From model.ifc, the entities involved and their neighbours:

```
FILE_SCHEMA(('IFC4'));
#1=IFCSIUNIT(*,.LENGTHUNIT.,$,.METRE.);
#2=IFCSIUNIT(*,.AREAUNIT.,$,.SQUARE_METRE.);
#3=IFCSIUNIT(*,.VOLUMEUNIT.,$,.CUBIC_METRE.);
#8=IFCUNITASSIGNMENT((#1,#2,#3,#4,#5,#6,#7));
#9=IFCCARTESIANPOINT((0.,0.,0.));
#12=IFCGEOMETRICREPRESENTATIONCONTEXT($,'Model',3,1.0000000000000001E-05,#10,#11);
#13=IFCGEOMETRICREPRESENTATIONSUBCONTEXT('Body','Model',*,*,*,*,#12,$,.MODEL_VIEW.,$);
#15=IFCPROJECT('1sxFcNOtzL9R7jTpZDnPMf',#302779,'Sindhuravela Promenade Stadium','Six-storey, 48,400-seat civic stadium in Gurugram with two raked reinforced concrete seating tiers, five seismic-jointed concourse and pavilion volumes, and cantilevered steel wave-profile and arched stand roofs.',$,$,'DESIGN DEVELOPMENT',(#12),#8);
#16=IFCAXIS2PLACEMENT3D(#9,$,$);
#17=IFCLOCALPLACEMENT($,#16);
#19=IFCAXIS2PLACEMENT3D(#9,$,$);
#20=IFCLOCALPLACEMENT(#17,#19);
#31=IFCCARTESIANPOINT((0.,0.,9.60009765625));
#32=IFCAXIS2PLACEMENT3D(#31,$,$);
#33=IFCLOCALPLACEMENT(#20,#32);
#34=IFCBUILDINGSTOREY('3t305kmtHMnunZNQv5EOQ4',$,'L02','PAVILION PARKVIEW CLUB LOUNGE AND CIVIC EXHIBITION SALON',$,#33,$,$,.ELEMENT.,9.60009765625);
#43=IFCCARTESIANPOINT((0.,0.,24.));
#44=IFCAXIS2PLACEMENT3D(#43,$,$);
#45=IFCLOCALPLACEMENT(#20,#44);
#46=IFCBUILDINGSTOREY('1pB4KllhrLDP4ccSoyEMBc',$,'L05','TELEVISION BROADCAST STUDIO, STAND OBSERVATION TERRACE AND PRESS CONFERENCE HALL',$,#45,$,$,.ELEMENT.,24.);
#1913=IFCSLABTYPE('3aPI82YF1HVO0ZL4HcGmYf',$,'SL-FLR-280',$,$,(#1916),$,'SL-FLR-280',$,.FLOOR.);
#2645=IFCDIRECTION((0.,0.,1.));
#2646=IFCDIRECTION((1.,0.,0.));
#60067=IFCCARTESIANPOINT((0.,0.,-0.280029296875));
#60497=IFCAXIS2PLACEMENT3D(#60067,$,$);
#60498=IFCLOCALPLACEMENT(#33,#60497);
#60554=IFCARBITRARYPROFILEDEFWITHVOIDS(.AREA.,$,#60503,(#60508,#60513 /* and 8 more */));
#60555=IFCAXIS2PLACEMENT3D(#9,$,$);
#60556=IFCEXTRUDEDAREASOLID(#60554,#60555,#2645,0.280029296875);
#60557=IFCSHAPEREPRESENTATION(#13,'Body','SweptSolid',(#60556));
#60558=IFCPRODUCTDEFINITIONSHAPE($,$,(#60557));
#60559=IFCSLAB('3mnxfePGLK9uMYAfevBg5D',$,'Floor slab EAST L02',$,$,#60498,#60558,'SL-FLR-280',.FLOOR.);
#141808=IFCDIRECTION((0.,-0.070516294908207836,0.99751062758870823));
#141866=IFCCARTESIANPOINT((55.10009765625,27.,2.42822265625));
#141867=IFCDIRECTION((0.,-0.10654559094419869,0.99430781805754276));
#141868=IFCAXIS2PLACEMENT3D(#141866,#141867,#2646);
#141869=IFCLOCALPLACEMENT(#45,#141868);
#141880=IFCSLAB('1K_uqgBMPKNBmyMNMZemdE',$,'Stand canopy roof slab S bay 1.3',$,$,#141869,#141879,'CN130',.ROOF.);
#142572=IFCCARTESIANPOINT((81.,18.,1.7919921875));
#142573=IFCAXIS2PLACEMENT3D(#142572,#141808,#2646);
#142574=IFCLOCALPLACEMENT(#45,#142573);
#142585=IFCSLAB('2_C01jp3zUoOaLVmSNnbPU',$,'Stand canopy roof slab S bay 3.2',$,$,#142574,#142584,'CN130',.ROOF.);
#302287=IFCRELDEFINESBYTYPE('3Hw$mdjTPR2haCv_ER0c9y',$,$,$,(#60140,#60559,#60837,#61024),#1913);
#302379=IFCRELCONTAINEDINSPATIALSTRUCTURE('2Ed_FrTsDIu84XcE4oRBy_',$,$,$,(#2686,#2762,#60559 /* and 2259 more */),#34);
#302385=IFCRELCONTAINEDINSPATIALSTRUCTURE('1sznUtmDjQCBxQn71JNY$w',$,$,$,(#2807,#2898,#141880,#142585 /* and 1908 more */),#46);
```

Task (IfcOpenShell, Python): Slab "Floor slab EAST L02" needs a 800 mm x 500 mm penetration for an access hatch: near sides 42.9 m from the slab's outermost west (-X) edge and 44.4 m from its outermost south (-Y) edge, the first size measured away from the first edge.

```python
import numpy as np
import ifcopenshell
import ifcopenshell.api.feature
import ifcopenshell.api.geometry
import ifcopenshell.api.root
import ifcopenshell.geom
import ifcopenshell.util.placement
import ifcopenshell.util.representation
import ifcopenshell.util.shape
import ifcopenshell.util.unit

model = ifcopenshell.open("model.ifc")
unit_scale = ifcopenshell.util.unit.calculate_unit_scale(model)
settings = ifcopenshell.geom.settings()


def volume(element):
    """Net volume in cubic metres, openings subtracted."""
    shape = ifcopenshell.geom.create_shape(settings, element)
    return ifcopenshell.util.shape.get_volume(shape.geometry)


slab = model.by_id(60559)
before = volume(slab)

# Extent in the slab's own axes, in metres. The edges named are its -X and -Y sides.
slab_shape = ifcopenshell.geom.create_shape(settings, slab)
vertices = ifcopenshell.util.shape.get_vertices(slab_shape.geometry)
x_min, y_min, bottom = vertices.min(axis=0)
top = vertices[:, 2].max()

opening = ifcopenshell.api.root.create_entity(model, ifc_class="IfcOpeningElement", name="Access hatch opening", predefined_type="OPENING")
context = ifcopenshell.util.representation.get_context(model, "Model", "Body", "MODEL_VIEW")
width, depth = 0.8, 0.5
outline = [(0.0, 0.0), (width, 0.0), (width, depth), (0.0, depth), (0.0, 0.0)]
# Overshoot both faces by 50 mm so the cut is clean.
shape = ifcopenshell.api.geometry.add_slab_representation(
    model, context=context, depth=top - bottom + 0.1, polyline=outline
)
ifcopenshell.api.geometry.assign_representation(model, product=opening, representation=shape)

matrix = ifcopenshell.util.placement.get_local_placement(slab.ObjectPlacement)
matrix[:, 3] = matrix @ np.append(np.array([x_min + 42.9, y_min + 44.4, bottom - 0.05]) / unit_scale, 1.0)
ifcopenshell.api.geometry.edit_object_placement(model, product=opening, matrix=matrix, is_si=False)
ifcopenshell.api.feature.add_feature(model, feature=opening, element=slab)

after = volume(slab)

print(f"slab volume {before:.3f} -> {after:.3f} m3")

model.write("model_edited.ifc")
```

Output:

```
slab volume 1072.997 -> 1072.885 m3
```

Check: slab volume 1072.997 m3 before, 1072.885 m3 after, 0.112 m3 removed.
